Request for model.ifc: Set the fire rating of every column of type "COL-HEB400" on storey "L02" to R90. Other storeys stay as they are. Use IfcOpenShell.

First a look at what the model holds.

```python
import ifcopenshell
import ifcopenshell.util.element

model = ifcopenshell.open("model.ifc")
print(model.schema)
storey = next(s for s in model.by_type("IfcBuildingStorey") if s.Name == "L02")
columns = [e for e in ifcopenshell.util.element.get_decomposition(storey) if e.is_a("IfcColumn")]
seen = {}
for e in columns:
    element_type = ifcopenshell.util.element.get_type(e)
    key = (element_type.Name if element_type != e and element_type else None, ifcopenshell.util.element.get_pset(e, "Pset_ColumnCommon", "FireRating"))
    seen[key] = seen.get(key, 0) + 1
for (name, value), count in sorted(seen.items(), key=str):
    print(count, "x", name, "|", value)
```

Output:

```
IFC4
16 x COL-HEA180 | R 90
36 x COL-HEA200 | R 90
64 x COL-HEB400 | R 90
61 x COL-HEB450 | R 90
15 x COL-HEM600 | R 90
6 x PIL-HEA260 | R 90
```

```python
import ifcopenshell
import ifcopenshell.api.pset
import ifcopenshell.util.element

model = ifcopenshell.open("model.ifc")

storey = next(s for s in model.by_type("IfcBuildingStorey") if s.Name == "L02")
columns = [e for e in ifcopenshell.util.element.get_decomposition(storey) if e.is_a("IfcColumn")]

count = 0
for e in columns:
    element_type = ifcopenshell.util.element.get_type(e)
    if element_type in (None, e) or element_type.Name != "COL-HEB400":
        continue
    # add_pset returns the element's existing set when there is one.
    pset = ifcopenshell.api.pset.add_pset(model, product=e, name="Pset_ColumnCommon")
    ifcopenshell.api.pset.edit_pset(model, pset=pset, properties={"FireRating": "R90"})
    count += 1

print(count, "columns updated")

model.write("model-out.ifc")
```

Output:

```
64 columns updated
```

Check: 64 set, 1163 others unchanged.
